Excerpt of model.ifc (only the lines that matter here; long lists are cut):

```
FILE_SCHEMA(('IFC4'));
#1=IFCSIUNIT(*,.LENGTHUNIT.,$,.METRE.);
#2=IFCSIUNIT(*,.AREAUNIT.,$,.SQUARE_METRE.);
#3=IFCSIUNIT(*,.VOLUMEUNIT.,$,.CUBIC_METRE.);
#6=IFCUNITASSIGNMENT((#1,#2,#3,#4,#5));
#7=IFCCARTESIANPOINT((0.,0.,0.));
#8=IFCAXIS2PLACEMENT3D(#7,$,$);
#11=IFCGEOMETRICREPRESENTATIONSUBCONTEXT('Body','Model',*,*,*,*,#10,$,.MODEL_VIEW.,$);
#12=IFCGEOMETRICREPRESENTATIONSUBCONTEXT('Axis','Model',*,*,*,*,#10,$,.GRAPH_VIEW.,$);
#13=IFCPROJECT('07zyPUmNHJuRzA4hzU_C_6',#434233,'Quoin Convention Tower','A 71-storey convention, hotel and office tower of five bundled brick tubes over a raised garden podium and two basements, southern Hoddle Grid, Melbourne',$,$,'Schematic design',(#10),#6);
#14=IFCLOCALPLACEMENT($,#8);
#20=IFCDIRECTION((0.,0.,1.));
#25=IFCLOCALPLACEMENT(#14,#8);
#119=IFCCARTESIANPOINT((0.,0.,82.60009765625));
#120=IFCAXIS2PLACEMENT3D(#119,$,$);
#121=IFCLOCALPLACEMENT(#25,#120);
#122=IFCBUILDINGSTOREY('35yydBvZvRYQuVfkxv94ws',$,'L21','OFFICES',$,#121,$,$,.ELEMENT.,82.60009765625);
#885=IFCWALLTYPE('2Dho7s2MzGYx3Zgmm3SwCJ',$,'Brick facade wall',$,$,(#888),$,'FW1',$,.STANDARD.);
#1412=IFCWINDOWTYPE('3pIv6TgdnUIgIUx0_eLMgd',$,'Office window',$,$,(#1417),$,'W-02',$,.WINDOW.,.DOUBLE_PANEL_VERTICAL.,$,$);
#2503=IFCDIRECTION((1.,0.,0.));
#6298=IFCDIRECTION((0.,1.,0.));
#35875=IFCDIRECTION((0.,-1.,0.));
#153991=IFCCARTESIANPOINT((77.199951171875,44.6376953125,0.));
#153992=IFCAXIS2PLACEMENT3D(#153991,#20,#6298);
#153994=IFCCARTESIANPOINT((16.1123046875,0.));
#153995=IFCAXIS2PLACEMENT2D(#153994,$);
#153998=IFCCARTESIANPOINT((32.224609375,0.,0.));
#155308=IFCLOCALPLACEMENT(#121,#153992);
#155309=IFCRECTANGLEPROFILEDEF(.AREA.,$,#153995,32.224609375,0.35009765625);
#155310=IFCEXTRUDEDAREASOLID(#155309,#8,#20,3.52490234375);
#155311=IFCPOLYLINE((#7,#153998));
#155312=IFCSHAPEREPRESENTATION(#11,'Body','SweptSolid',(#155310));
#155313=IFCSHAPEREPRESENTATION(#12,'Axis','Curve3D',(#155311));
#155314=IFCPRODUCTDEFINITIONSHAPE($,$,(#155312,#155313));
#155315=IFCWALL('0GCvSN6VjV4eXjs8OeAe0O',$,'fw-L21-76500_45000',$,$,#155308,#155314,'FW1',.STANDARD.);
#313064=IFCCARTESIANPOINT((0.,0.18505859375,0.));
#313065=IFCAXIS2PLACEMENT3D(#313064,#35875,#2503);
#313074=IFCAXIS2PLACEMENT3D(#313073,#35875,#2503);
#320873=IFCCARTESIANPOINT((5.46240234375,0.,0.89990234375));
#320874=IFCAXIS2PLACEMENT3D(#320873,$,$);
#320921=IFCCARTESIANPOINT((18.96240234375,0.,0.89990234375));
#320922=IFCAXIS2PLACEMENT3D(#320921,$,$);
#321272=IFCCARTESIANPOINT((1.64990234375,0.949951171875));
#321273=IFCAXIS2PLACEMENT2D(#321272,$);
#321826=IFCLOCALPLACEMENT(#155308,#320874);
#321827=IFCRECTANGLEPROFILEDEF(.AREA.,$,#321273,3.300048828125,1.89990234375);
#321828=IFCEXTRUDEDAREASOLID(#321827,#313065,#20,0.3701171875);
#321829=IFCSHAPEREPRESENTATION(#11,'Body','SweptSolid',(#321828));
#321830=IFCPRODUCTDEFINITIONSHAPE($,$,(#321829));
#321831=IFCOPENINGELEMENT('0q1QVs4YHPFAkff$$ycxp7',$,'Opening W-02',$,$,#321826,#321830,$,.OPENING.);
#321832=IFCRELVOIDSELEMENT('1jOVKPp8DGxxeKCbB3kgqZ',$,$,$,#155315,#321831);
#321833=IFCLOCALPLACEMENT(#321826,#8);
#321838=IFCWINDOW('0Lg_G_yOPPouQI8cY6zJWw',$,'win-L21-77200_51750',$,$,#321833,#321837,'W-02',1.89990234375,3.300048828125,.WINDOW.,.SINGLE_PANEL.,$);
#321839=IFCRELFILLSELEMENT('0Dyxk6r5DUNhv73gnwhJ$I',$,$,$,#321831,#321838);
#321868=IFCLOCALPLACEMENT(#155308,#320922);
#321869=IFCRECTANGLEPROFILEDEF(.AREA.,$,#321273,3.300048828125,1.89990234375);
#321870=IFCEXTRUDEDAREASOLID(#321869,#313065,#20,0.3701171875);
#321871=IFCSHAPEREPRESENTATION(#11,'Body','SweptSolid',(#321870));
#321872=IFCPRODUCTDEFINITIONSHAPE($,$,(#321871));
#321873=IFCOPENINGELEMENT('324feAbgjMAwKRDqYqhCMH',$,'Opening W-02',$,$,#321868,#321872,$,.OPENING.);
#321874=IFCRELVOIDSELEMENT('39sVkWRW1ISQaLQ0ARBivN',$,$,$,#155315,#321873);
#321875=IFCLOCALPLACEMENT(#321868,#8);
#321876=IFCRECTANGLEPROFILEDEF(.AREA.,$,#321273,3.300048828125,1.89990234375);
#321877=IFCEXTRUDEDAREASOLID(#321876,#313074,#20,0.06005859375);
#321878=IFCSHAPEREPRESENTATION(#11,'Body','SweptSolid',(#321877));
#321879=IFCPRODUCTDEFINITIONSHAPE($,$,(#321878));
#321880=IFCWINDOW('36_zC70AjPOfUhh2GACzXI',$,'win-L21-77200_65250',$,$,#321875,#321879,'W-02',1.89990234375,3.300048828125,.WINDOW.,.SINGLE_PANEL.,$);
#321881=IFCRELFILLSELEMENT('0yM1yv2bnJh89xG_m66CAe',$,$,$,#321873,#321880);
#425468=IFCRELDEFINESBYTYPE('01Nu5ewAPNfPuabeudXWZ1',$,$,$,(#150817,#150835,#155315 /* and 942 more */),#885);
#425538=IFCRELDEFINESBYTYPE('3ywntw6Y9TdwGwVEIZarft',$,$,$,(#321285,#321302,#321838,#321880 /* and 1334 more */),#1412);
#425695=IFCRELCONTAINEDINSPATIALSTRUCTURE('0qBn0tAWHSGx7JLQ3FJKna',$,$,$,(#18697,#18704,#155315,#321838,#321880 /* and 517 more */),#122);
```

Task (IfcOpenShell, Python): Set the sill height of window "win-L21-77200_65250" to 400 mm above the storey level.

```python
import numpy as np
import ifcopenshell
import ifcopenshell.api.geometry
import ifcopenshell.geom
import ifcopenshell.util.element
import ifcopenshell.util.placement
import ifcopenshell.util.shape
import ifcopenshell.util.unit

model = ifcopenshell.open("model.ifc")
unit_scale = ifcopenshell.util.unit.calculate_unit_scale(model)

window = model.by_guid("36_zC70AjPOfUhh2GACzXI")
opening = window.FillsVoids[0].RelatingOpeningElement
storey = ifcopenshell.util.element.get_container(window, ifc_class="IfcBuildingStorey")
level = ifcopenshell.util.placement.get_local_placement(storey.ObjectPlacement)[2, 3]

# The opening's origin need not be at the sill, so measure its lowest point.
shape = ifcopenshell.geom.create_shape(ifcopenshell.geom.settings(), opening)
bottom = ifcopenshell.util.shape.get_shape_bottom_elevation(shape, shape.geometry) / unit_scale
dz = level + 0.4 / unit_scale - bottom

shift = np.array([0.0, 0.0, dz])
# The window is placed relative to its opening, so it follows when the opening moves.
matrix = ifcopenshell.util.placement.get_local_placement(opening.ObjectPlacement)
matrix[:3, 3] += shift
ifcopenshell.api.geometry.edit_object_placement(
    model, product=opening, matrix=matrix, is_si=False, should_transform_children=True
)

print(f"moved by {dz * unit_scale:+.3f} m")

model.write("model-out.ifc")
```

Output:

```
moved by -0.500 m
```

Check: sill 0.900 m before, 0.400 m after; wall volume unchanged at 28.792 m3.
